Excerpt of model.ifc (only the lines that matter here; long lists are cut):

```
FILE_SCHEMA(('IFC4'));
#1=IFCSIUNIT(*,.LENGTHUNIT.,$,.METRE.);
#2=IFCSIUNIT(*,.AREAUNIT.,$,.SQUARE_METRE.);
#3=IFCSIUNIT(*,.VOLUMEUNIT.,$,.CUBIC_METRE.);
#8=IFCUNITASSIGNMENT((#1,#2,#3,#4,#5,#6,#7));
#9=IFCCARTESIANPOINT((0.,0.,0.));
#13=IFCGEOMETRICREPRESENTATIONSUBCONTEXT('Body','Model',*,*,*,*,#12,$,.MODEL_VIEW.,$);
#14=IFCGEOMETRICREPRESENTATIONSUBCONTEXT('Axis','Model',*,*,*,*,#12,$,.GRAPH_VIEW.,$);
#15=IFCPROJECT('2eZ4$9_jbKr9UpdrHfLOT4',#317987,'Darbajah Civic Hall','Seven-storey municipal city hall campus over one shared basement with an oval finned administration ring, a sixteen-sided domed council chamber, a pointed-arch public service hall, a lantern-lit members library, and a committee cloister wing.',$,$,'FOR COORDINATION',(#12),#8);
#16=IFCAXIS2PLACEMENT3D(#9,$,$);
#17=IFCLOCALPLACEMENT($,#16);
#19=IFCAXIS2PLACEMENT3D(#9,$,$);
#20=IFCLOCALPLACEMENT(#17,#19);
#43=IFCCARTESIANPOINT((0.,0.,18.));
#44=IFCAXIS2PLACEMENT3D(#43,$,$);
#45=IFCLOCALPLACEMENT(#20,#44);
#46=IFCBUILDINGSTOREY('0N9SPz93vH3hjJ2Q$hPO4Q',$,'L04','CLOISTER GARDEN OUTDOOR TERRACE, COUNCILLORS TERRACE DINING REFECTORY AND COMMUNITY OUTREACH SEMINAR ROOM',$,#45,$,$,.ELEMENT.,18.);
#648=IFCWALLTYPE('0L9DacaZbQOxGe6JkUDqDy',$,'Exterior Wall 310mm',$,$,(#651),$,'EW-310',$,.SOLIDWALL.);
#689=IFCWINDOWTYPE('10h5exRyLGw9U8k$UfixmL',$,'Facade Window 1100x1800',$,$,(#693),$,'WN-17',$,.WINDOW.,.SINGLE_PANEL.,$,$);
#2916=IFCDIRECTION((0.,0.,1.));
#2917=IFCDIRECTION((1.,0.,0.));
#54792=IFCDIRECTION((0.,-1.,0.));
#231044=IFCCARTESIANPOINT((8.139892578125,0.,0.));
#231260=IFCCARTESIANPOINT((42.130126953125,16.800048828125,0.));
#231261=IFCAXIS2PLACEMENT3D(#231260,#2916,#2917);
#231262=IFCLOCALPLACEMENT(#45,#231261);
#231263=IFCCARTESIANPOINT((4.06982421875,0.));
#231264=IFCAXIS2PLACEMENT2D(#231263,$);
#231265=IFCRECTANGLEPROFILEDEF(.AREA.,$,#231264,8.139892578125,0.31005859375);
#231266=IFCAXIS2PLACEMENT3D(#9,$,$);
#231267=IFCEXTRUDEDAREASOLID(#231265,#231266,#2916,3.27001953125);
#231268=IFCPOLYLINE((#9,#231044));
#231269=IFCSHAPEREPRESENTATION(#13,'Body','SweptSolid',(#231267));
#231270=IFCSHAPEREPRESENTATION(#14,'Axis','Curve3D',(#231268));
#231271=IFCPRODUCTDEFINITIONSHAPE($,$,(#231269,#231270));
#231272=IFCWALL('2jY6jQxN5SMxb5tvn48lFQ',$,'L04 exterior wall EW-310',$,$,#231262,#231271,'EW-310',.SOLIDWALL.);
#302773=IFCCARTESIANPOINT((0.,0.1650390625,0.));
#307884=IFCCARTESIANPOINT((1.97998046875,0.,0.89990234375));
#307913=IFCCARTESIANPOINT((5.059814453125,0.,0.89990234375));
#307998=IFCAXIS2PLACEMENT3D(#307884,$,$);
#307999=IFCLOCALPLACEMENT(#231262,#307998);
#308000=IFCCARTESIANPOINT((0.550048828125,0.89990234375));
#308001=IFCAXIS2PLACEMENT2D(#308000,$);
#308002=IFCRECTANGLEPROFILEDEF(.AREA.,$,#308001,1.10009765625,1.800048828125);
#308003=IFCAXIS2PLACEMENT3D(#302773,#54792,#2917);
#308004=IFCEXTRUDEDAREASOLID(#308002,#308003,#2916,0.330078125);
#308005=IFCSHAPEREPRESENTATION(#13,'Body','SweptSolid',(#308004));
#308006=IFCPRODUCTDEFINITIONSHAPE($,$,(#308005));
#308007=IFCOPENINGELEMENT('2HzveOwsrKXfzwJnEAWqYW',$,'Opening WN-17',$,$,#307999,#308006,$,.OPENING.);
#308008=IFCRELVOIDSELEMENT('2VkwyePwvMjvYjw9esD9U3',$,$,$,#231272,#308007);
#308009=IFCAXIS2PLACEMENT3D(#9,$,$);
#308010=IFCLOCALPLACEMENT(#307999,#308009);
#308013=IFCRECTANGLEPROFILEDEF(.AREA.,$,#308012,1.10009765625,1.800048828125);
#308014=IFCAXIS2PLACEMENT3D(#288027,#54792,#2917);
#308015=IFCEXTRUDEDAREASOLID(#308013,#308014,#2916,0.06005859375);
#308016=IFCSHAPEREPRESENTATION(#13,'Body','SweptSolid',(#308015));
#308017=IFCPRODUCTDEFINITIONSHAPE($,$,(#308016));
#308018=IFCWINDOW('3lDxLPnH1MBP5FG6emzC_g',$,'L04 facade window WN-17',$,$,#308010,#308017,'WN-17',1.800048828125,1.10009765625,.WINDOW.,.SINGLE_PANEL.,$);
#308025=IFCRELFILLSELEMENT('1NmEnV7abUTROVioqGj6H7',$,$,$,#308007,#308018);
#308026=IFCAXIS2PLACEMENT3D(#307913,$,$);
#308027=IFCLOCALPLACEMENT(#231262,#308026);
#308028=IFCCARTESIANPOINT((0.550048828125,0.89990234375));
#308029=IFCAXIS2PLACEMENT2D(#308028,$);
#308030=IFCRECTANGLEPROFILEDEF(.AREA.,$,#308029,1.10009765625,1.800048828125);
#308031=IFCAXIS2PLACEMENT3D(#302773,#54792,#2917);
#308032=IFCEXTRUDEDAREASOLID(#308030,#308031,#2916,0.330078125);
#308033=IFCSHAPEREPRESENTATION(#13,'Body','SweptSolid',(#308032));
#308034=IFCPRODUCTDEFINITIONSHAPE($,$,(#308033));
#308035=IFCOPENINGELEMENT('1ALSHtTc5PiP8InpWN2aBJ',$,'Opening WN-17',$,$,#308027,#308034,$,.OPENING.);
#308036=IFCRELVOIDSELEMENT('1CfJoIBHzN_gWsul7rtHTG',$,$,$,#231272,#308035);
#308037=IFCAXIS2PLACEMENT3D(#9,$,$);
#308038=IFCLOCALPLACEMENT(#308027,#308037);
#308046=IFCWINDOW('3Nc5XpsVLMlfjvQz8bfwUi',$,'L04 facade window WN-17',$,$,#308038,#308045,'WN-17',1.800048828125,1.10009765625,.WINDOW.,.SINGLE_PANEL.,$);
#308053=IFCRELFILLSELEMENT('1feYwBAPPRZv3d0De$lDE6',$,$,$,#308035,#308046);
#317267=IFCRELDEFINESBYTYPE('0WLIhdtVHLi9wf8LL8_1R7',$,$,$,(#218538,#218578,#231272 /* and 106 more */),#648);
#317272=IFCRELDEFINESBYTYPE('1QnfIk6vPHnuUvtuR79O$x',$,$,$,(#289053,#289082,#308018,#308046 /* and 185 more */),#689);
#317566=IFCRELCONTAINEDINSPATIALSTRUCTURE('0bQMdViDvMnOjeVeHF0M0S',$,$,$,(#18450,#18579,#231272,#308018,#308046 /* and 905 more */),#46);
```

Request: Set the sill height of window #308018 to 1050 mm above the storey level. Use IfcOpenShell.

```python
import numpy as np
import ifcopenshell
import ifcopenshell.api.geometry
import ifcopenshell.geom
import ifcopenshell.util.element
import ifcopenshell.util.placement
import ifcopenshell.util.shape
import ifcopenshell.util.unit

model = ifcopenshell.open("model.ifc")
unit_scale = ifcopenshell.util.unit.calculate_unit_scale(model)

window = model.by_id(308018)
opening = window.FillsVoids[0].RelatingOpeningElement
storey = ifcopenshell.util.element.get_container(window, ifc_class="IfcBuildingStorey")
level = ifcopenshell.util.placement.get_local_placement(storey.ObjectPlacement)[2, 3]

# The opening's origin need not be at the sill, so measure its lowest point.
shape = ifcopenshell.geom.create_shape(ifcopenshell.geom.settings(), opening)
bottom = ifcopenshell.util.shape.get_shape_bottom_elevation(shape, shape.geometry) / unit_scale
dz = level + 1.05 - bottom

shift = np.array([0.0, 0.0, dz])
# The window is placed relative to its opening, so it follows when the opening moves.
matrix = ifcopenshell.util.placement.get_local_placement(opening.ObjectPlacement)
matrix[:3, 3] += shift
ifcopenshell.api.geometry.edit_object_placement(
    model, product=opening, matrix=matrix, is_si=False, should_transform_children=True
)

print(f"moved by {dz * unit_scale:+.3f} m")

model.write("model_rev.ifc")
```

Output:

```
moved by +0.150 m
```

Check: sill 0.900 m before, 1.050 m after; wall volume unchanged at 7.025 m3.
